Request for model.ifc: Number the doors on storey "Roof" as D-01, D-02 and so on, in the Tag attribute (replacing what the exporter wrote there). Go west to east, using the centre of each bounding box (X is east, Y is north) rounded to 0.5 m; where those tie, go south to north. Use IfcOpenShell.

First a look at what the model holds.

```python
import ifcopenshell
import ifcopenshell.util.element
import ifcopenshell.util.placement

model = ifcopenshell.open("model.ifc")
print(model.schema)
storey = next(s for s in model.by_type("IfcBuildingStorey") if s.Name == "Roof")
doors = [e for e in ifcopenshell.util.element.get_decomposition(storey) if e.is_a("IfcDoor")]
for e in sorted(doors, key=lambda e: e.id()):
    origin = ifcopenshell.util.placement.get_local_placement(e.ObjectPlacement)[:3, 3]
    print(e.id(), e.Tag, e.Name, origin.round(2) + 0.0, sep=" | ")
```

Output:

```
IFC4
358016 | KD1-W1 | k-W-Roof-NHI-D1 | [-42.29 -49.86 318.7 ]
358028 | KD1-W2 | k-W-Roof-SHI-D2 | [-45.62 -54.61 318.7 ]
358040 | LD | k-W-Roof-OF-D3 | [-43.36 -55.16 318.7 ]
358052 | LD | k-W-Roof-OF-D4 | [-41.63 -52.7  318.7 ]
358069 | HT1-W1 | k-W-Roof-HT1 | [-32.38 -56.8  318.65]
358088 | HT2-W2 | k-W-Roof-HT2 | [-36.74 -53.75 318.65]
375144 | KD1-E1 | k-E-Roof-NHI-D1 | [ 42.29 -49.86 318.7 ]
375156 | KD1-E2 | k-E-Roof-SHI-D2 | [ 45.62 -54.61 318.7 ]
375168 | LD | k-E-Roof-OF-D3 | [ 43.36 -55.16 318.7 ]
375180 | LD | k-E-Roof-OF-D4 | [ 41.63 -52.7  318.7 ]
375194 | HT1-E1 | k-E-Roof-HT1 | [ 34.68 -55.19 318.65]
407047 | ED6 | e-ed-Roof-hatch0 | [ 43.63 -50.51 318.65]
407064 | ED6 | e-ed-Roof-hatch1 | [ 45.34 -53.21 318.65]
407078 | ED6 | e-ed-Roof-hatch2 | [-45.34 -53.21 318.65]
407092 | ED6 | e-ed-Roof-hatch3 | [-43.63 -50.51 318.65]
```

```python
import ifcopenshell
import ifcopenshell.geom
import ifcopenshell.util.element
import ifcopenshell.util.shape

model = ifcopenshell.open("model.ifc")
settings = ifcopenshell.geom.settings()
settings.set("use-world-coords", True)


def centre(element):
    shape = ifcopenshell.geom.create_shape(settings, element)
    return ifcopenshell.util.shape.get_bbox_centroid(shape.geometry)


storey = next(s for s in model.by_type("IfcBuildingStorey") if s.Name == "Roof")
doors = [e for e in ifcopenshell.util.element.get_decomposition(storey) if e.is_a("IfcDoor")]

# Insertion points can sit at a corner or the storey origin, so sort by the geometry (in metres).
centres = {e: centre(e) for e in doors}
doors.sort(key=lambda e: (round(centres[e][0] / 0.5), centres[e][1]))

for i, e in enumerate(doors, start=1):
    number = f"D-{i:02d}"
    e.Tag = number
    print(e.id(), number)

model.write("model_v2.ifc")
```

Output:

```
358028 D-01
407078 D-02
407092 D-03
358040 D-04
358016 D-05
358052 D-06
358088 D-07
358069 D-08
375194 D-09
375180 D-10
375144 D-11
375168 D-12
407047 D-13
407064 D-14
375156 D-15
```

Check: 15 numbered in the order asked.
